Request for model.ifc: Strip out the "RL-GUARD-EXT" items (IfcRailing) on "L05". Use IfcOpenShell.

First a look at what the model holds.

```python
import ifcopenshell
import ifcopenshell.util.element

model = ifcopenshell.open("model.ifc")
print(model.schema)
storey = next(s for s in model.by_type("IfcBuildingStorey") if s.Name == "L05")
railings = [e for e in ifcopenshell.util.element.get_decomposition(storey) if e.is_a("IfcRailing")]
seen = {}
for e in railings:
    element_type = ifcopenshell.util.element.get_type(e)
    name = element_type.Name if element_type not in (None, e) else None
    seen[name] = seen.get(name, 0) + 1
for name, count in sorted(seen.items(), key=str):
    print(count, "x", name)
```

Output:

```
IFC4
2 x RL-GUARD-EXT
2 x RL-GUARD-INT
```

```python
import ifcopenshell
import ifcopenshell.api.root
import ifcopenshell.util.element

model = ifcopenshell.open("model.ifc")

storey = next(s for s in model.by_type("IfcBuildingStorey") if s.Name == "L05")
railings = [e for e in ifcopenshell.util.element.get_decomposition(storey) if e.is_a("IfcRailing")]
targets = [e for e in railings if (t := ifcopenshell.util.element.get_type(e)) not in (None, e) and t.Name == "RL-GUARD-EXT"]

for e in targets:
    ifcopenshell.api.root.remove_product(model, product=e)
print(len(targets), "removed")

model.write("model-out.ifc")
```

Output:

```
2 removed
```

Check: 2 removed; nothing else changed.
